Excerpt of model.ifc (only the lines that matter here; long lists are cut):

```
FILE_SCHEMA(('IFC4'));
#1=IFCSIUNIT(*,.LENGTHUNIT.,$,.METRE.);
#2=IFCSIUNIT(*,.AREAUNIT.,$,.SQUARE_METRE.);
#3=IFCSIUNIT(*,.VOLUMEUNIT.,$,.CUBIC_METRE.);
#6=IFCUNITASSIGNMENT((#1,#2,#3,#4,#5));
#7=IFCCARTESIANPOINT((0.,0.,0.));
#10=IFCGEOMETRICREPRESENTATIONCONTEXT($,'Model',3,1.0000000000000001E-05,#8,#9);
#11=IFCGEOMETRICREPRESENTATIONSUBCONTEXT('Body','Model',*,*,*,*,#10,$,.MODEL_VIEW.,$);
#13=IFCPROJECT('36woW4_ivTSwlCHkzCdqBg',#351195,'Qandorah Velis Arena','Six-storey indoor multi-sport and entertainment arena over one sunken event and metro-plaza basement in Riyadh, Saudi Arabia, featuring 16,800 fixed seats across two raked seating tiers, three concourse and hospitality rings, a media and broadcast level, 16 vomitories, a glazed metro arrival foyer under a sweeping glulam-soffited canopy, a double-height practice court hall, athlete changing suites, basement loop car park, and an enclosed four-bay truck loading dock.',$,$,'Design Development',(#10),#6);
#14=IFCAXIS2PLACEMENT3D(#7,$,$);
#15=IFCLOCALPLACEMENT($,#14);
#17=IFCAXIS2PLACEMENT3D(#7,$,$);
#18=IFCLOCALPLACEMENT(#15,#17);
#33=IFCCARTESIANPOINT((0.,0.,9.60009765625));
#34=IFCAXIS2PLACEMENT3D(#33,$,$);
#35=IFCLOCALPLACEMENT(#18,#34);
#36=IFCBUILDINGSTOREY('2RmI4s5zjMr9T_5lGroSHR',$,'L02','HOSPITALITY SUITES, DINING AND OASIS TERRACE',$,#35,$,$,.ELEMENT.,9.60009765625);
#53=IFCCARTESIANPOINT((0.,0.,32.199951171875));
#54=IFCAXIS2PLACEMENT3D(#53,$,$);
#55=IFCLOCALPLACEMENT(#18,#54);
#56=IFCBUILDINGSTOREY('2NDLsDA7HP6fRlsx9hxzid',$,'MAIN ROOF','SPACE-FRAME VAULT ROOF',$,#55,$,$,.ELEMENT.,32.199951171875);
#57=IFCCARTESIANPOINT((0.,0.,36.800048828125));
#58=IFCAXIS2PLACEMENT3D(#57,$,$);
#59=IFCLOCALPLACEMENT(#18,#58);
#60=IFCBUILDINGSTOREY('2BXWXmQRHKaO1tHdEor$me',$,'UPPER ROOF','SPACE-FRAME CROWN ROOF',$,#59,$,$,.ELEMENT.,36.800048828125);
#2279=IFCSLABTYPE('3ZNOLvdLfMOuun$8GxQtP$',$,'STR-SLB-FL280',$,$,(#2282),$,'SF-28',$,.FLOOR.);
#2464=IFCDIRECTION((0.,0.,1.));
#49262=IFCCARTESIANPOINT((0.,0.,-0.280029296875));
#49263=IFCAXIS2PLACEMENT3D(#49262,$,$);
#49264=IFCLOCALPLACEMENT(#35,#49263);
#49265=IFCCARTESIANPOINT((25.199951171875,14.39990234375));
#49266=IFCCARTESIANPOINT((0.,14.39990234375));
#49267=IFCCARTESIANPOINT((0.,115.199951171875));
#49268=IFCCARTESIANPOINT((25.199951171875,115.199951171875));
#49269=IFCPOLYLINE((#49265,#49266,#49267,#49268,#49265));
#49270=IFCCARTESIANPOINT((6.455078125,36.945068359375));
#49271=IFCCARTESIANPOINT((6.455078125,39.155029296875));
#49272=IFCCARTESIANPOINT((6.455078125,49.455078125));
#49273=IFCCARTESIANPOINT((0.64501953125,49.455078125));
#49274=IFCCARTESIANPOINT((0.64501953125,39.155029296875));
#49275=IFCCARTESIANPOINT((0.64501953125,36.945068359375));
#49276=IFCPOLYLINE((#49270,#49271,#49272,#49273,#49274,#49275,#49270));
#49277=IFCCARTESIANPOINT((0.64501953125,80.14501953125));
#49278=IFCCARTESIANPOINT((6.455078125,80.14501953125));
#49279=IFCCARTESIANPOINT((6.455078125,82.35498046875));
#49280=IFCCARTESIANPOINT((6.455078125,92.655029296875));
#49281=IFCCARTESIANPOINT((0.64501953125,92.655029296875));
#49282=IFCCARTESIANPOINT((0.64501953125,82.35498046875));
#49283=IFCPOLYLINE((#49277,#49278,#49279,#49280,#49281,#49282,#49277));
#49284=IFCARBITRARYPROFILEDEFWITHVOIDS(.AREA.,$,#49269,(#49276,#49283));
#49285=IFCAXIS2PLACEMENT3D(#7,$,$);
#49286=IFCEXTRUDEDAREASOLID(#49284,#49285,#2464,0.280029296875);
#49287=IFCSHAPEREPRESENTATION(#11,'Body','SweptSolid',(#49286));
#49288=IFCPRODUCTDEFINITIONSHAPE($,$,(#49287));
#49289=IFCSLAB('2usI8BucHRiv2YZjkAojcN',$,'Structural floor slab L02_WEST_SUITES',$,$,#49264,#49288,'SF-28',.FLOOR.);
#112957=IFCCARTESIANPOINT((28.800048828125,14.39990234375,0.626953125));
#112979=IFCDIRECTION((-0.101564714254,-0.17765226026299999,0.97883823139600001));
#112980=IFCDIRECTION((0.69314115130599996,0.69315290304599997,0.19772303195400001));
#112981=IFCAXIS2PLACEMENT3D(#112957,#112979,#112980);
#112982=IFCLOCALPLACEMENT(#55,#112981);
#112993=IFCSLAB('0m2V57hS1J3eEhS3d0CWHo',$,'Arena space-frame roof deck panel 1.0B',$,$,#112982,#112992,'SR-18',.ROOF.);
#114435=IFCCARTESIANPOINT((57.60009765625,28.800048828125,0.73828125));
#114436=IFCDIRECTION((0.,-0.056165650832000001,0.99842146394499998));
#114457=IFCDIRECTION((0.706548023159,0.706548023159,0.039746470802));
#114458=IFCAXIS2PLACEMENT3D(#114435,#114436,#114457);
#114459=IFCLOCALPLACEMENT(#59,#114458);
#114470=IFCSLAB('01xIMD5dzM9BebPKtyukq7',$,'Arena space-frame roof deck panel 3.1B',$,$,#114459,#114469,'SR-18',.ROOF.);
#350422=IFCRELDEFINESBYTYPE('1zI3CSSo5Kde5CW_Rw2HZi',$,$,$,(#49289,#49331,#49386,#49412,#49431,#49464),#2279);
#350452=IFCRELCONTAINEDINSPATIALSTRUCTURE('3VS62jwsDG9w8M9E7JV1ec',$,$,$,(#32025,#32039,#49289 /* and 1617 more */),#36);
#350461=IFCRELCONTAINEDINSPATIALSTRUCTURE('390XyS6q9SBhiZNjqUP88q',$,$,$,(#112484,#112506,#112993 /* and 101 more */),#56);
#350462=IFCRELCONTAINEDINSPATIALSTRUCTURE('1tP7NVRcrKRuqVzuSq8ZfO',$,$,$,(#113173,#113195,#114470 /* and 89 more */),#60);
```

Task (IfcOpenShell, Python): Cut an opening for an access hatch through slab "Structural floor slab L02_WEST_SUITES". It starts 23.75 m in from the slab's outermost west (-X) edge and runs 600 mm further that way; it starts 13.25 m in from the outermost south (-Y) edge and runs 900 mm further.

```python
import numpy as np
import ifcopenshell
import ifcopenshell.api.feature
import ifcopenshell.api.geometry
import ifcopenshell.api.root
import ifcopenshell.geom
import ifcopenshell.util.placement
import ifcopenshell.util.representation
import ifcopenshell.util.shape
import ifcopenshell.util.unit

model = ifcopenshell.open("model.ifc")
unit_scale = ifcopenshell.util.unit.calculate_unit_scale(model)
settings = ifcopenshell.geom.settings()


def volume(element):
    """Net volume in cubic metres, openings subtracted."""
    shape = ifcopenshell.geom.create_shape(settings, element)
    return ifcopenshell.util.shape.get_volume(shape.geometry)


slab = model.by_id(49289)
before = volume(slab)

# Extent in the slab's own axes, in metres. The edges named are its -X and -Y sides.
slab_shape = ifcopenshell.geom.create_shape(settings, slab)
vertices = ifcopenshell.util.shape.get_vertices(slab_shape.geometry)
x_min, y_min, bottom = vertices.min(axis=0)
top = vertices[:, 2].max()

opening = ifcopenshell.api.root.create_entity(model, ifc_class="IfcOpeningElement", name="Access hatch opening", predefined_type="OPENING")
context = ifcopenshell.util.representation.get_context(model, "Model", "Body", "MODEL_VIEW")
width, depth = 0.6, 0.9
outline = [(0.0, 0.0), (width, 0.0), (width, depth), (0.0, depth), (0.0, 0.0)]
# Overshoot both faces by 50 mm so the cut is clean.
shape = ifcopenshell.api.geometry.add_slab_representation(
    model, context=context, depth=top - bottom + 0.1, polyline=outline
)
ifcopenshell.api.geometry.assign_representation(model, product=opening, representation=shape)

matrix = ifcopenshell.util.placement.get_local_placement(slab.ObjectPlacement)
matrix[:, 3] = matrix @ np.append(np.array([x_min + 23.75, y_min + 13.25, bottom - 0.05]) / unit_scale, 1.0)
ifcopenshell.api.geometry.edit_object_placement(model, product=opening, matrix=matrix, is_si=False)
ifcopenshell.api.feature.add_feature(model, feature=opening, element=slab)

after = volume(slab)

print(f"slab volume {before:.3f} -> {after:.3f} m3")

model.write("model-out.ifc")
```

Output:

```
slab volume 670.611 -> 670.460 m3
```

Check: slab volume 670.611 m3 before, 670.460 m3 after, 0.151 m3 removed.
